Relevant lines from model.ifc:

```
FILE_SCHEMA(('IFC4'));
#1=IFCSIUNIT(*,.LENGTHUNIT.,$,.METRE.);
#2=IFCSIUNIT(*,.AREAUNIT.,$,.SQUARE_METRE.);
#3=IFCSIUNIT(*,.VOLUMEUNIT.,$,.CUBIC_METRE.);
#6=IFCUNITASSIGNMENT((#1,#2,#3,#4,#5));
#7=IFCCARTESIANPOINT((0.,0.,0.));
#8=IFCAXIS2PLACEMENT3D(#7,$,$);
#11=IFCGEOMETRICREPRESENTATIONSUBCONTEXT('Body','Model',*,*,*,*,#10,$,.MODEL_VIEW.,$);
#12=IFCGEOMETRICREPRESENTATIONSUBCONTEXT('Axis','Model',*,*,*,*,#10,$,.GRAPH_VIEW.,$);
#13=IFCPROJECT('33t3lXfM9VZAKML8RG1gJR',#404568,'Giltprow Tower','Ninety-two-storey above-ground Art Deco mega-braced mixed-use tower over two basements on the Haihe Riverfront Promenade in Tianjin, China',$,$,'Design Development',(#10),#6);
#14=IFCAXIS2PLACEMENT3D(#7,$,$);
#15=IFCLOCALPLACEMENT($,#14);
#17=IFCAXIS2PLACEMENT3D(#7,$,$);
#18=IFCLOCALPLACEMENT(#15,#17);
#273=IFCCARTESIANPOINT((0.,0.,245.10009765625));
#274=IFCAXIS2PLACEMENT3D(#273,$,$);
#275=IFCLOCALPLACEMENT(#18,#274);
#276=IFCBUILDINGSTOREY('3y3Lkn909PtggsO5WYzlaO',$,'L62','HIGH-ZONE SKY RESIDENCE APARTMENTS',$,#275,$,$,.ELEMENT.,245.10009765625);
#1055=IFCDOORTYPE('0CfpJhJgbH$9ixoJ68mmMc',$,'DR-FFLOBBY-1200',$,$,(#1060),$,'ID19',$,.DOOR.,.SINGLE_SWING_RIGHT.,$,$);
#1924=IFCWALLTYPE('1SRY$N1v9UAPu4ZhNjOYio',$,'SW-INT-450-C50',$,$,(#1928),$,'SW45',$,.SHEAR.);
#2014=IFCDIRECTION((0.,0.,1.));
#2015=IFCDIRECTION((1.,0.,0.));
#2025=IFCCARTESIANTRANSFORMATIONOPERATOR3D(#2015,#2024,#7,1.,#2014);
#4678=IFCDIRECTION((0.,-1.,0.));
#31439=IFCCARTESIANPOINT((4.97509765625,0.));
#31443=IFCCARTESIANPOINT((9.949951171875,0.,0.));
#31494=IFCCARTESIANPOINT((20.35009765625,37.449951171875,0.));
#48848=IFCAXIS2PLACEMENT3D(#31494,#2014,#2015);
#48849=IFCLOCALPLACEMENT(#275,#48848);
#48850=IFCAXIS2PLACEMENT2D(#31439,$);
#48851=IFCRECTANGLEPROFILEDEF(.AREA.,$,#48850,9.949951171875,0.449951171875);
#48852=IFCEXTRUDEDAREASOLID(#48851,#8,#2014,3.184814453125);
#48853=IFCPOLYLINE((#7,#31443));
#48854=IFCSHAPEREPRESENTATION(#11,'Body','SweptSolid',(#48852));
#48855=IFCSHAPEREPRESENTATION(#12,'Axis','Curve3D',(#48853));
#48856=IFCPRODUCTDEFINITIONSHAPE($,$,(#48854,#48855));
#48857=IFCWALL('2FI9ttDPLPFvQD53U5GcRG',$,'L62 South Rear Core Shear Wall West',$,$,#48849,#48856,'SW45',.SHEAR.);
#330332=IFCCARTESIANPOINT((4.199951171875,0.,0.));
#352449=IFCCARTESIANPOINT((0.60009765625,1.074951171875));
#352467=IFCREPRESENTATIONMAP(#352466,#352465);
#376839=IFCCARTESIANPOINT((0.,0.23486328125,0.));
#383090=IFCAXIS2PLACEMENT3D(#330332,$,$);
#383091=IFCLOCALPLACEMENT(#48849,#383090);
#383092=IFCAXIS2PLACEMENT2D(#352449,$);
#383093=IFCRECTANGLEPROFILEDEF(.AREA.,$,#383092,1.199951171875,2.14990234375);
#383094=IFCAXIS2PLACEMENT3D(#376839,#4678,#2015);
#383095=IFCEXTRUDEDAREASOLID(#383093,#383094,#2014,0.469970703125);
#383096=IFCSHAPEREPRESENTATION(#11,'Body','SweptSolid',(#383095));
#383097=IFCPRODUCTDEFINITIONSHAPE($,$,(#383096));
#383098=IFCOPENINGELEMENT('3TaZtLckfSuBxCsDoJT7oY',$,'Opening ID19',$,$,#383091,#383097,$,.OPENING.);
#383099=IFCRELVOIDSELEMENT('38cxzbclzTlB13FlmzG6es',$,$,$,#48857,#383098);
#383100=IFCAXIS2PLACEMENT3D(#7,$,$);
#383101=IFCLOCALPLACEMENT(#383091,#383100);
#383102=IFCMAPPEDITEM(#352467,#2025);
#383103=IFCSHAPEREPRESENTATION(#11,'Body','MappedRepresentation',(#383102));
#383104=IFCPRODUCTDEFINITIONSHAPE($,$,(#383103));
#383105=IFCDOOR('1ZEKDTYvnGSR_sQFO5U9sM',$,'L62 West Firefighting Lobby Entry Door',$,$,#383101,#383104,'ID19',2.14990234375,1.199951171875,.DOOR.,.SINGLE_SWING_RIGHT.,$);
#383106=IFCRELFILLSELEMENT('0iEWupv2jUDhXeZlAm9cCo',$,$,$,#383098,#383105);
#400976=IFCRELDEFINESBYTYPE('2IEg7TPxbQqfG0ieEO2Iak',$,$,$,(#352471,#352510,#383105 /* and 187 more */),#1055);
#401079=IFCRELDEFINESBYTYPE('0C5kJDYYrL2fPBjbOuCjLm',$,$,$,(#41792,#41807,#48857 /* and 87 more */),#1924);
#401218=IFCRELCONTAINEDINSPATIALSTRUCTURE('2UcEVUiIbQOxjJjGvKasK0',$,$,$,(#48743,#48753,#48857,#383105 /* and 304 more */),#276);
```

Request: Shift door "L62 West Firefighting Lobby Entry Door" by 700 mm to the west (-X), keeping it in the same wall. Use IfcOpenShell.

```python
import ifcopenshell
import ifcopenshell.api.geometry
import ifcopenshell.util.placement

model = ifcopenshell.open("model.ifc")

door = model.by_guid("1ZEKDTYvnGSR_sQFO5U9sM")
opening = door.FillsVoids[0].RelatingOpeningElement
wall = opening.VoidsElements[0].RelatingBuildingElement

wall_matrix = ifcopenshell.util.placement.get_local_placement(wall.ObjectPlacement)
shift = wall_matrix[:3, 0] * -0.7
before = ifcopenshell.util.placement.get_local_placement(door.ObjectPlacement)[:3, 3].copy()

# The door is placed relative to its opening, so it follows when the opening moves.
matrix = ifcopenshell.util.placement.get_local_placement(opening.ObjectPlacement)
matrix[:3, 3] += shift
ifcopenshell.api.geometry.edit_object_placement(
    model, product=opening, matrix=matrix, is_si=False, should_transform_children=True
)

after = ifcopenshell.util.placement.get_local_placement(door.ObjectPlacement)[:3, 3]
print("door moved by", (after - before).round(3) + 0.0)

model.write("model-out.ifc")
```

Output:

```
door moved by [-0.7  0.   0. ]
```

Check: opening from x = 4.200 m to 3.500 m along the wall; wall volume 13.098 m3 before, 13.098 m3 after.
